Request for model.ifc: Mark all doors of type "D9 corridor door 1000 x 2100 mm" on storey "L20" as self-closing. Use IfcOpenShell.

First a look at what the model holds.

```python
import ifcopenshell
import ifcopenshell.util.element

model = ifcopenshell.open("model.ifc")
print(model.schema)
storey = next(s for s in model.by_type("IfcBuildingStorey") if s.Name == "L20")
doors = [e for e in ifcopenshell.util.element.get_decomposition(storey) if e.is_a("IfcDoor")]
seen = {}
for e in doors:
    element_type = ifcopenshell.util.element.get_type(e)
    key = (element_type.Name if element_type != e and element_type else None, ifcopenshell.util.element.get_pset(e, "Pset_DoorCommon", "SelfClosing"))
    seen[key] = seen.get(key, 0) + 1
for (name, value), count in sorted(seen.items(), key=str):
    print(count, "x", name, "|", value)
```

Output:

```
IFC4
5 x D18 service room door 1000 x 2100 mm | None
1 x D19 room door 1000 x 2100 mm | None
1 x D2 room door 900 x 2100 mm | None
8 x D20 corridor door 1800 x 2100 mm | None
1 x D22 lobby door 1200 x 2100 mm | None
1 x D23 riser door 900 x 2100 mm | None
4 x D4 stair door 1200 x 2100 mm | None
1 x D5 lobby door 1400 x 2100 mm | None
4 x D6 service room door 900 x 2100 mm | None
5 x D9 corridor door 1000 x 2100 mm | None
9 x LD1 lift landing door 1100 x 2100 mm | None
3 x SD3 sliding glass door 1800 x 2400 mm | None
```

```python
import ifcopenshell
import ifcopenshell.api.pset
import ifcopenshell.util.element

model = ifcopenshell.open("model.ifc")

storey = next(s for s in model.by_type("IfcBuildingStorey") if s.Name == "L20")
doors = [e for e in ifcopenshell.util.element.get_decomposition(storey) if e.is_a("IfcDoor")]

count = 0
for e in doors:
    element_type = ifcopenshell.util.element.get_type(e)
    if element_type in (None, e) or element_type.Name != "D9 corridor door 1000 x 2100 mm":
        continue
    # add_pset returns the element's existing set when there is one.
    pset = ifcopenshell.api.pset.add_pset(model, product=e, name="Pset_DoorCommon")
    ifcopenshell.api.pset.edit_pset(model, pset=pset, properties={"SelfClosing": True})
    count += 1

print(count, "doors updated")

model.write("model_edited.ifc")
```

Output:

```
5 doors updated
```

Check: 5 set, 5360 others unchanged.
